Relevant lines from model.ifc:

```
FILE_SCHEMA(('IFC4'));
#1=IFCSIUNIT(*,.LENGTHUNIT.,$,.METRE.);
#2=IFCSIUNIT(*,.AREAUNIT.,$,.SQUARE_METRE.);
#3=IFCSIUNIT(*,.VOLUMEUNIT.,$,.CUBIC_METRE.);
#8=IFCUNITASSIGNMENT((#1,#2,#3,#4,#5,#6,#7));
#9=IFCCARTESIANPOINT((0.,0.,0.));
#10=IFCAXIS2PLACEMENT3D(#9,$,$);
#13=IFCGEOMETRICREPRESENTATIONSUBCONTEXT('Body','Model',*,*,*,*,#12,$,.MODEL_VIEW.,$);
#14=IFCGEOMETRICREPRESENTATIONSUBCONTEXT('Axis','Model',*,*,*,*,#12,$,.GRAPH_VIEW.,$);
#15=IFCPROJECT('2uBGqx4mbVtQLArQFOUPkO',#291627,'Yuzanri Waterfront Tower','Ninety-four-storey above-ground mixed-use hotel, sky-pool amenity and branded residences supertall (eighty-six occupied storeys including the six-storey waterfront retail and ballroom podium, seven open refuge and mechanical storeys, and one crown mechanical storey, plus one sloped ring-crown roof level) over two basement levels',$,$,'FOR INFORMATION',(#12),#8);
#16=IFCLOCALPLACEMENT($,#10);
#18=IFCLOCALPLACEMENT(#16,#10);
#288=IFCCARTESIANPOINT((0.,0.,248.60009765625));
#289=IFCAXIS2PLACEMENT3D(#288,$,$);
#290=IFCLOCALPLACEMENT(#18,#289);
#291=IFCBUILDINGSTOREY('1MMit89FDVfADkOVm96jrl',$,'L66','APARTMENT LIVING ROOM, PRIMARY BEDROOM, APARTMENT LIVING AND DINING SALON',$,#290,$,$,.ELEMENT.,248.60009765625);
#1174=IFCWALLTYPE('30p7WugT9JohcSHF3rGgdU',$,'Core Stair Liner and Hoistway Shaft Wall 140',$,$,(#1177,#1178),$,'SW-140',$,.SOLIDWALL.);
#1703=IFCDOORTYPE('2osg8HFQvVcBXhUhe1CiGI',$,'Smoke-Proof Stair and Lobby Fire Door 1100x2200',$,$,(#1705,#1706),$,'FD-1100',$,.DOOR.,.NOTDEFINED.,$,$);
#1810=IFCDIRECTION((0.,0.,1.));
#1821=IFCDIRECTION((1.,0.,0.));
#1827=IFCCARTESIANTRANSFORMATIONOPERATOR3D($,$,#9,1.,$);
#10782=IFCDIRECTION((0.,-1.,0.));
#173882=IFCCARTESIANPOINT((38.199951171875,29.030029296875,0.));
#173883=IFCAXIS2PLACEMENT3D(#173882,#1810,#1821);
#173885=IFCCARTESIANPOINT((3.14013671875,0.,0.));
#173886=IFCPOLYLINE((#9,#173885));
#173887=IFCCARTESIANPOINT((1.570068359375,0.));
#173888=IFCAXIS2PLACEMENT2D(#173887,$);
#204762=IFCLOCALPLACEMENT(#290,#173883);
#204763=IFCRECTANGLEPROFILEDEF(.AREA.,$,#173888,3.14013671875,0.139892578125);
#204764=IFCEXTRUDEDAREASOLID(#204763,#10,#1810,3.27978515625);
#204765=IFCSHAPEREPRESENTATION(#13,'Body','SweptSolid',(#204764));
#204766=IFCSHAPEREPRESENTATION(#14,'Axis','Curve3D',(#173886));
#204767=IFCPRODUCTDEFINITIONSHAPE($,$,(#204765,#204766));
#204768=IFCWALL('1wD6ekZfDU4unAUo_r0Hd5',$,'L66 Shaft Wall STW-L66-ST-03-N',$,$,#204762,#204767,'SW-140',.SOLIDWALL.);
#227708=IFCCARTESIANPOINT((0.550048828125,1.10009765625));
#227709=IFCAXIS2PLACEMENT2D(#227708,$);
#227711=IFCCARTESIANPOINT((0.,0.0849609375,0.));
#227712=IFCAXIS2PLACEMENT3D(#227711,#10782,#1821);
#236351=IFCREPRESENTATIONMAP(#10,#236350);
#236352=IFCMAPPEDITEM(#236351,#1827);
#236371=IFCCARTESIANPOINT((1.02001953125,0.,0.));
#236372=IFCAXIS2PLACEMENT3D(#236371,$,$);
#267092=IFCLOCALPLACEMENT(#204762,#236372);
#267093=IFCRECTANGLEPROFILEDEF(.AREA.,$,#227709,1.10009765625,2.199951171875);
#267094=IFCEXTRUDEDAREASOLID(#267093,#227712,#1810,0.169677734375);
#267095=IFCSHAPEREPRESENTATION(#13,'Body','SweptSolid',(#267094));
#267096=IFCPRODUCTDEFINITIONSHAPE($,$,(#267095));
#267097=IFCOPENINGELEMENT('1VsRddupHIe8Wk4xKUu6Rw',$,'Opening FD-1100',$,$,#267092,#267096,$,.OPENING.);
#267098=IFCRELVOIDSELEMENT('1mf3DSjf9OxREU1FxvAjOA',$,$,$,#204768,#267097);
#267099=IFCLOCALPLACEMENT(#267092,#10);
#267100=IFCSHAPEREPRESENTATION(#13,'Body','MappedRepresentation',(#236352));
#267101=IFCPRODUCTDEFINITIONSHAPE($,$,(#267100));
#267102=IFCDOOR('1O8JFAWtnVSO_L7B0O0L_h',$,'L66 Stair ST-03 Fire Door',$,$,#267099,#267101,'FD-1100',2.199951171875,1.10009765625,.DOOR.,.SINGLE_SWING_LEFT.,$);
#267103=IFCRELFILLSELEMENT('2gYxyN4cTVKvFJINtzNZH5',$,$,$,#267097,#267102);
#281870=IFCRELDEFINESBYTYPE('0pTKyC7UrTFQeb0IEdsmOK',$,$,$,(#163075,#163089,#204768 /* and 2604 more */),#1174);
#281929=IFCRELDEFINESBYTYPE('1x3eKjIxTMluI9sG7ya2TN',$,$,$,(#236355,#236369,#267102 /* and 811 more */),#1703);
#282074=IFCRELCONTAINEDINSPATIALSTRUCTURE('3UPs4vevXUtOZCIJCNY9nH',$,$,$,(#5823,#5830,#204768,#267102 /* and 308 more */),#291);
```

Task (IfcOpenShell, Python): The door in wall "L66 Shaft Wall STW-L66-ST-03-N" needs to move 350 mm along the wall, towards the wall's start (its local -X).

```python
import ifcopenshell
import ifcopenshell.api.geometry
import ifcopenshell.util.placement
import ifcopenshell.util.unit

model = ifcopenshell.open("model.ifc")
unit_scale = ifcopenshell.util.unit.calculate_unit_scale(model)

door = model.by_guid("1O8JFAWtnVSO_L7B0O0L_h")
opening = door.FillsVoids[0].RelatingOpeningElement
wall = opening.VoidsElements[0].RelatingBuildingElement

wall_matrix = ifcopenshell.util.placement.get_local_placement(wall.ObjectPlacement)
shift = wall_matrix[:3, 0] * -0.35 / unit_scale
before = ifcopenshell.util.placement.get_local_placement(door.ObjectPlacement)[:3, 3].copy()

# The door is placed relative to its opening, so it follows when the opening moves.
matrix = ifcopenshell.util.placement.get_local_placement(opening.ObjectPlacement)
matrix[:3, 3] += shift
ifcopenshell.api.geometry.edit_object_placement(
    model, product=opening, matrix=matrix, is_si=False, should_transform_children=True
)

after = ifcopenshell.util.placement.get_local_placement(door.ObjectPlacement)[:3, 3]
print("door moved by", (after - before).round(3) + 0.0)

model.write("model_edited.ifc")
```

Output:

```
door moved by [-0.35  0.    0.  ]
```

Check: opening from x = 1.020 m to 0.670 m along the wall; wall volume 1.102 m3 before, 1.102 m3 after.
